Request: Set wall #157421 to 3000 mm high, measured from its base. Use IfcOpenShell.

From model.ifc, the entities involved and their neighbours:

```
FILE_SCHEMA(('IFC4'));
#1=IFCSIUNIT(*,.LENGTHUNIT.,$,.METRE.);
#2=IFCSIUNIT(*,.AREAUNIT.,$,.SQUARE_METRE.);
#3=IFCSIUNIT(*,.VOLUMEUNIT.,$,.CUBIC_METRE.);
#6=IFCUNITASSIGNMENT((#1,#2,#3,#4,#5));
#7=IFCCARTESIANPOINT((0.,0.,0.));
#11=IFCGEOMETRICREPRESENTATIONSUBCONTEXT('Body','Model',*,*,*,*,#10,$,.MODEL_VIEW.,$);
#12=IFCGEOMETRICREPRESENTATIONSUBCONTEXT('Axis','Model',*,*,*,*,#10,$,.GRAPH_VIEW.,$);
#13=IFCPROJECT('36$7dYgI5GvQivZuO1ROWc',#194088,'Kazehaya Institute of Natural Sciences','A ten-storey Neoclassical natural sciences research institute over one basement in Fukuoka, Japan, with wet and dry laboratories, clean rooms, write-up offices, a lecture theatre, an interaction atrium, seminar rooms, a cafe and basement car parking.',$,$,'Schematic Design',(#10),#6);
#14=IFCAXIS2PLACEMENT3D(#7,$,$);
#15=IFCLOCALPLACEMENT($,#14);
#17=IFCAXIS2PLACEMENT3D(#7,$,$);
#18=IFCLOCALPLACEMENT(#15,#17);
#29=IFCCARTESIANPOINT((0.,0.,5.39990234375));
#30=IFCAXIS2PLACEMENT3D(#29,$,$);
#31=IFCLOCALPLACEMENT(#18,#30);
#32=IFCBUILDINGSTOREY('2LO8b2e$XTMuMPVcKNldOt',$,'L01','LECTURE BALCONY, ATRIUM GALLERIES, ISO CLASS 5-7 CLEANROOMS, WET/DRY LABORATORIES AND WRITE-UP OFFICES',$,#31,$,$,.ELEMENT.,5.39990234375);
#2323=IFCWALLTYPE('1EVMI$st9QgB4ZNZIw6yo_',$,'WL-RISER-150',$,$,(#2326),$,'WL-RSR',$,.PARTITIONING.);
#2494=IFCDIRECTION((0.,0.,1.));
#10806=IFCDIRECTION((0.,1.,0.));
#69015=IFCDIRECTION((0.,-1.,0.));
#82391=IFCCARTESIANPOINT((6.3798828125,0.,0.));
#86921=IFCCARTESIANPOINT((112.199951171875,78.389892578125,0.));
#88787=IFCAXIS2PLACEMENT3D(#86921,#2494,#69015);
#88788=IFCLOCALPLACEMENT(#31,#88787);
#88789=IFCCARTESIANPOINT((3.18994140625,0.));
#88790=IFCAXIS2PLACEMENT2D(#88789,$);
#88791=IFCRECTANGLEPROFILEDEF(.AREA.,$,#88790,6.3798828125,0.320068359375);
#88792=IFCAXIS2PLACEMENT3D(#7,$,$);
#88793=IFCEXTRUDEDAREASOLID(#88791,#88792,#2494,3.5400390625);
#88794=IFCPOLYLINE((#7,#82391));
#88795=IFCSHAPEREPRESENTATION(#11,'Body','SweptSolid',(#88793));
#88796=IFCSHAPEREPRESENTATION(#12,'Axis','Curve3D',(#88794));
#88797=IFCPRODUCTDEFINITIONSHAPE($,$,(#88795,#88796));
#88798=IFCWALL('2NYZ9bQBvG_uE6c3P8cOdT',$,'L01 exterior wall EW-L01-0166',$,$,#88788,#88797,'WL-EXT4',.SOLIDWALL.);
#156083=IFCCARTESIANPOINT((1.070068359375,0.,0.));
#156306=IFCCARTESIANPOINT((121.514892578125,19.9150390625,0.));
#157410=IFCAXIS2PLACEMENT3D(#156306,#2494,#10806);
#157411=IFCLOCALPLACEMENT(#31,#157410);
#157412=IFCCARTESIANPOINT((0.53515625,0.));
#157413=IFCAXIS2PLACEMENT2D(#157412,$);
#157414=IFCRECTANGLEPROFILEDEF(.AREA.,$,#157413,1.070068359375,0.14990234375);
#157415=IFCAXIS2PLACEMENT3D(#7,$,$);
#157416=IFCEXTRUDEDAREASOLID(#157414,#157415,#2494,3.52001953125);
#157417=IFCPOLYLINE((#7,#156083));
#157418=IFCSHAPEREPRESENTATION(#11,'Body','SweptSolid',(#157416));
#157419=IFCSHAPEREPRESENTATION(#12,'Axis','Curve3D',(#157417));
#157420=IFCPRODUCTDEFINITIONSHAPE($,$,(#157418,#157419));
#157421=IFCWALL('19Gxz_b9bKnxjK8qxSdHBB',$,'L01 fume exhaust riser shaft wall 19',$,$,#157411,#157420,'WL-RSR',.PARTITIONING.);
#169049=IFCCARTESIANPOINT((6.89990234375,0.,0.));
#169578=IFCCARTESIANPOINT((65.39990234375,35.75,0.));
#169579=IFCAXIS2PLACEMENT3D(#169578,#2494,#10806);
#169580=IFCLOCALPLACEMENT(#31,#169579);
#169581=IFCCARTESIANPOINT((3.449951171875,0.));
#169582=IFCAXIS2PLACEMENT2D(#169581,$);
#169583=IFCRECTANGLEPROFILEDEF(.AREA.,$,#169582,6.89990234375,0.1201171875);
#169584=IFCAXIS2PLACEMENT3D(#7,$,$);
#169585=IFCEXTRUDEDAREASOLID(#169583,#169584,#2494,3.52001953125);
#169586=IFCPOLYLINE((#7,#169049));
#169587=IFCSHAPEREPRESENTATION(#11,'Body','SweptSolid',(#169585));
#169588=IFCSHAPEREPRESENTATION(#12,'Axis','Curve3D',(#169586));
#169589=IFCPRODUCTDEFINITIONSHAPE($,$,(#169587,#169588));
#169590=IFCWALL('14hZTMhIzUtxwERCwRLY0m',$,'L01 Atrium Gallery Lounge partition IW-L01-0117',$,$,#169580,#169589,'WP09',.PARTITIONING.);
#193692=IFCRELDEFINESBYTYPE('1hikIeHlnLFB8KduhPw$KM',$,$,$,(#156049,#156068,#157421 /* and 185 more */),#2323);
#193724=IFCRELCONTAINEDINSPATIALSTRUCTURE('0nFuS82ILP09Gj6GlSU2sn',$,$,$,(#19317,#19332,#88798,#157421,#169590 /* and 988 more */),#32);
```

```python
import ifcopenshell
import ifcopenshell.geom
import ifcopenshell.util.representation
import ifcopenshell.util.shape
import ifcopenshell.util.unit

model = ifcopenshell.open("model.ifc")
unit_scale = ifcopenshell.util.unit.calculate_unit_scale(model)
settings = ifcopenshell.geom.settings()


def volume(element):
    """Net volume in cubic metres, openings subtracted."""
    shape = ifcopenshell.geom.create_shape(settings, element)
    return ifcopenshell.util.shape.get_volume(shape.geometry)


wall = model.by_id(157421)
before = volume(wall)

body = ifcopenshell.util.representation.get_representation(wall, "Model", "Body")
solid = body.Items[0]
old_height = solid.Depth
solid.Depth = 3 / unit_scale
after = volume(wall)

print(f"height {old_height:g} -> {solid.Depth:g}, volume {before:.3f} -> {after:.3f} m3")

model.write("model_v2.ifc")
```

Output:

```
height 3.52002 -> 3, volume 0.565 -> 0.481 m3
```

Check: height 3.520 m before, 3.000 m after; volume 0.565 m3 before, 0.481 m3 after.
